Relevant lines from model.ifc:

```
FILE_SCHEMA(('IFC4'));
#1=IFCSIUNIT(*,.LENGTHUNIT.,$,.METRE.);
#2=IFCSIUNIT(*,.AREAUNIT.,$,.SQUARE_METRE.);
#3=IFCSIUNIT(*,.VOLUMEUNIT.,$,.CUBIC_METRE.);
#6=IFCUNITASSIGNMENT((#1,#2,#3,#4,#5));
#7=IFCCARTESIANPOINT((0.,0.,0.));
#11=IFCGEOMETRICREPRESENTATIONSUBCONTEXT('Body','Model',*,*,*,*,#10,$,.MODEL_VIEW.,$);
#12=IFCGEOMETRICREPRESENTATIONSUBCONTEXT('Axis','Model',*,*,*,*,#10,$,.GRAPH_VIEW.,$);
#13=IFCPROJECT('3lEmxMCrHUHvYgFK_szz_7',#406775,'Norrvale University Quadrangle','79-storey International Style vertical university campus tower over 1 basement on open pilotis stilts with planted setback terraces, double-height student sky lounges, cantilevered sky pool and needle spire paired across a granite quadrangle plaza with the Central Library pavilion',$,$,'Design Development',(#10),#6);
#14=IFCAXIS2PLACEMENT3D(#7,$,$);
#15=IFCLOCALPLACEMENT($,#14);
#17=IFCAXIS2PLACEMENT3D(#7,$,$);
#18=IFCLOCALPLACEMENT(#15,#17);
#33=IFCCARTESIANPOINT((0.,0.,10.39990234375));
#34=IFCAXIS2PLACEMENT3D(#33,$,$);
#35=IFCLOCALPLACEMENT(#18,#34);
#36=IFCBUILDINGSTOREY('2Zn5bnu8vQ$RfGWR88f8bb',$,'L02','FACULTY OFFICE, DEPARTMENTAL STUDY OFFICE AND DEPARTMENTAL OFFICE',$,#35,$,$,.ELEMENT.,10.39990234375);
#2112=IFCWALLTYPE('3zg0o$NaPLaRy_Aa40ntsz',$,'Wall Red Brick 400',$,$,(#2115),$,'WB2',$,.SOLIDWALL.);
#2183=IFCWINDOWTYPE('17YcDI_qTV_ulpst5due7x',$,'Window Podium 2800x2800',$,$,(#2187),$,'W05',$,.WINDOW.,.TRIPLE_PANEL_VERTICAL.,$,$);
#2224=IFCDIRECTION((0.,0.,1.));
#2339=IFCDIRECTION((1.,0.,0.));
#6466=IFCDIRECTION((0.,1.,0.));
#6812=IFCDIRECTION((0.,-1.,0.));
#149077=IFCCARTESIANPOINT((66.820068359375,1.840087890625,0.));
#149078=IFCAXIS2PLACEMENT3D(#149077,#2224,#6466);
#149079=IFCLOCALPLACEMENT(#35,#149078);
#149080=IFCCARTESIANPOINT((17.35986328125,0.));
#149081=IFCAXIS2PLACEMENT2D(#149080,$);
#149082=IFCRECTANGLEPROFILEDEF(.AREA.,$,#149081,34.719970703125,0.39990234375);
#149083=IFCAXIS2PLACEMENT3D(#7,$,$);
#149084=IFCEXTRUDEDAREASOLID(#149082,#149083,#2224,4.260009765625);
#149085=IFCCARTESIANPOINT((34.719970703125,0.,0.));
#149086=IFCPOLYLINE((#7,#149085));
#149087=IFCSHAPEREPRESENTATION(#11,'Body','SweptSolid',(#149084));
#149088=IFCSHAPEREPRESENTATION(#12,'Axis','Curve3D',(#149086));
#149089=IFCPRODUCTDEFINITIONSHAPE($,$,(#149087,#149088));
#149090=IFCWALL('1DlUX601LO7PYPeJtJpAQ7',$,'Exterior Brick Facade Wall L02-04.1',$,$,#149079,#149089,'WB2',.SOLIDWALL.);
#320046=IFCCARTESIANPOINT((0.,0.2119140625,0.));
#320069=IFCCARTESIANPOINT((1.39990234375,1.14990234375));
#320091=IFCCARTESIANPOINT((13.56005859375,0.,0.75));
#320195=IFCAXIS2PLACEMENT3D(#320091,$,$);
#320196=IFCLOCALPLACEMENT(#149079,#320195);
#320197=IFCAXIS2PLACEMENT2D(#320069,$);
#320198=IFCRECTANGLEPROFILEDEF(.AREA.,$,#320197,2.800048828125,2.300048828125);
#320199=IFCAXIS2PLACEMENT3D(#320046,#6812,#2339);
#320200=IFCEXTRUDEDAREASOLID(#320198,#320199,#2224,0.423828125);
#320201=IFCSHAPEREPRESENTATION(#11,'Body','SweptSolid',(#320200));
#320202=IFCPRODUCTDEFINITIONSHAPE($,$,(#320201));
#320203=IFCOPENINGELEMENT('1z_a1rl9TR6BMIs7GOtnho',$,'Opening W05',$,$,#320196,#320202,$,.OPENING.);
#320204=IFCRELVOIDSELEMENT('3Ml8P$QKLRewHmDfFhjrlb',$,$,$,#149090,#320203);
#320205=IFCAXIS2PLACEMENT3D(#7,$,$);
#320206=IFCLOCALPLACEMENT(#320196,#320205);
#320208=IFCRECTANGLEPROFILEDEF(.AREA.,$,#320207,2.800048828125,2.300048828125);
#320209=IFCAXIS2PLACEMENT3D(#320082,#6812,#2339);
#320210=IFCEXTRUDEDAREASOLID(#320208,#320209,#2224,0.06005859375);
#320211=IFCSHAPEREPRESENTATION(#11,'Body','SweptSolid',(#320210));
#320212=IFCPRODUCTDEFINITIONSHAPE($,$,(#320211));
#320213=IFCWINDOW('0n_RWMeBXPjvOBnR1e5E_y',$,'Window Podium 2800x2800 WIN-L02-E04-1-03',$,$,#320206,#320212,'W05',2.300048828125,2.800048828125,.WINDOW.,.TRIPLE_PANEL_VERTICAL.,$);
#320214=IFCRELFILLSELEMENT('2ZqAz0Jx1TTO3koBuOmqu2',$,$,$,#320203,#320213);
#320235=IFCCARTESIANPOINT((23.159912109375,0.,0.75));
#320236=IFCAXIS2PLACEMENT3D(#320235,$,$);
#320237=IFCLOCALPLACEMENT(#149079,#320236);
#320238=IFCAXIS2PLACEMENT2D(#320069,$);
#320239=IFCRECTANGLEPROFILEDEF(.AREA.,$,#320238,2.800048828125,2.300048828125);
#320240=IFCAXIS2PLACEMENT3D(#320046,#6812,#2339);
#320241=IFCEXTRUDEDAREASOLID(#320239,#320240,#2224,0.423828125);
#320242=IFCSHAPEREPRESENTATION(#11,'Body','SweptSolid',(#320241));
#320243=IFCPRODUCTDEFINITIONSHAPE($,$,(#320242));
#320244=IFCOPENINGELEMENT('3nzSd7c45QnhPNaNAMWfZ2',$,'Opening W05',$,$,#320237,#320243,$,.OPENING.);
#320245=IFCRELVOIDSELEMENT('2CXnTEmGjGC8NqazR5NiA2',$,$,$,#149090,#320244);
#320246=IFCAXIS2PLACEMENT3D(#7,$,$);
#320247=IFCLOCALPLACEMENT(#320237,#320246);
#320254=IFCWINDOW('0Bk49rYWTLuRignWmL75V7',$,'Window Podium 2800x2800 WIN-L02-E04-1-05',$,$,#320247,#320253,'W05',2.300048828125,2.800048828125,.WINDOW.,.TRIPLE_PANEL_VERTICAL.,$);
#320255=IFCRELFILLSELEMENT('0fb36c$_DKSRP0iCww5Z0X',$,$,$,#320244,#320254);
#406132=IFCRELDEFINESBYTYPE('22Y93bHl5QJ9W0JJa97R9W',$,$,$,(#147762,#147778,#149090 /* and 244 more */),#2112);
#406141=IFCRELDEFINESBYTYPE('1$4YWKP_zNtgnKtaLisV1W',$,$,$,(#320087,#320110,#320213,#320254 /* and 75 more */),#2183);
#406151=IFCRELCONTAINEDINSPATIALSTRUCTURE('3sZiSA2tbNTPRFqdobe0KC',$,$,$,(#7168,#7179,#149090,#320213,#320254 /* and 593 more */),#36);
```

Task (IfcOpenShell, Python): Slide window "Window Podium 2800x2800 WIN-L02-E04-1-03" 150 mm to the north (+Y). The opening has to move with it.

```python
import ifcopenshell
import ifcopenshell.api.geometry
import ifcopenshell.util.placement
import ifcopenshell.util.unit

model = ifcopenshell.open("model.ifc")
unit_scale = ifcopenshell.util.unit.calculate_unit_scale(model)

window = model.by_guid("0n_RWMeBXPjvOBnR1e5E_y")
opening = window.FillsVoids[0].RelatingOpeningElement
wall = opening.VoidsElements[0].RelatingBuildingElement

wall_matrix = ifcopenshell.util.placement.get_local_placement(wall.ObjectPlacement)
shift = wall_matrix[:3, 0] * 0.15 / unit_scale
before = ifcopenshell.util.placement.get_local_placement(window.ObjectPlacement)[:3, 3].copy()

# The window is placed relative to its opening, so it follows when the opening moves.
matrix = ifcopenshell.util.placement.get_local_placement(opening.ObjectPlacement)
matrix[:3, 3] += shift
ifcopenshell.api.geometry.edit_object_placement(
    model, product=opening, matrix=matrix, is_si=False, should_transform_children=True
)

after = ifcopenshell.util.placement.get_local_placement(window.ObjectPlacement)[:3, 3]
print("window moved by", (after - before).round(3) + 0.0)

model.write("model_v2.ifc")
```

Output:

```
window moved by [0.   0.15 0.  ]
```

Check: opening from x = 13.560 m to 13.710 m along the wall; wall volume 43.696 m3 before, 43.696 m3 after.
